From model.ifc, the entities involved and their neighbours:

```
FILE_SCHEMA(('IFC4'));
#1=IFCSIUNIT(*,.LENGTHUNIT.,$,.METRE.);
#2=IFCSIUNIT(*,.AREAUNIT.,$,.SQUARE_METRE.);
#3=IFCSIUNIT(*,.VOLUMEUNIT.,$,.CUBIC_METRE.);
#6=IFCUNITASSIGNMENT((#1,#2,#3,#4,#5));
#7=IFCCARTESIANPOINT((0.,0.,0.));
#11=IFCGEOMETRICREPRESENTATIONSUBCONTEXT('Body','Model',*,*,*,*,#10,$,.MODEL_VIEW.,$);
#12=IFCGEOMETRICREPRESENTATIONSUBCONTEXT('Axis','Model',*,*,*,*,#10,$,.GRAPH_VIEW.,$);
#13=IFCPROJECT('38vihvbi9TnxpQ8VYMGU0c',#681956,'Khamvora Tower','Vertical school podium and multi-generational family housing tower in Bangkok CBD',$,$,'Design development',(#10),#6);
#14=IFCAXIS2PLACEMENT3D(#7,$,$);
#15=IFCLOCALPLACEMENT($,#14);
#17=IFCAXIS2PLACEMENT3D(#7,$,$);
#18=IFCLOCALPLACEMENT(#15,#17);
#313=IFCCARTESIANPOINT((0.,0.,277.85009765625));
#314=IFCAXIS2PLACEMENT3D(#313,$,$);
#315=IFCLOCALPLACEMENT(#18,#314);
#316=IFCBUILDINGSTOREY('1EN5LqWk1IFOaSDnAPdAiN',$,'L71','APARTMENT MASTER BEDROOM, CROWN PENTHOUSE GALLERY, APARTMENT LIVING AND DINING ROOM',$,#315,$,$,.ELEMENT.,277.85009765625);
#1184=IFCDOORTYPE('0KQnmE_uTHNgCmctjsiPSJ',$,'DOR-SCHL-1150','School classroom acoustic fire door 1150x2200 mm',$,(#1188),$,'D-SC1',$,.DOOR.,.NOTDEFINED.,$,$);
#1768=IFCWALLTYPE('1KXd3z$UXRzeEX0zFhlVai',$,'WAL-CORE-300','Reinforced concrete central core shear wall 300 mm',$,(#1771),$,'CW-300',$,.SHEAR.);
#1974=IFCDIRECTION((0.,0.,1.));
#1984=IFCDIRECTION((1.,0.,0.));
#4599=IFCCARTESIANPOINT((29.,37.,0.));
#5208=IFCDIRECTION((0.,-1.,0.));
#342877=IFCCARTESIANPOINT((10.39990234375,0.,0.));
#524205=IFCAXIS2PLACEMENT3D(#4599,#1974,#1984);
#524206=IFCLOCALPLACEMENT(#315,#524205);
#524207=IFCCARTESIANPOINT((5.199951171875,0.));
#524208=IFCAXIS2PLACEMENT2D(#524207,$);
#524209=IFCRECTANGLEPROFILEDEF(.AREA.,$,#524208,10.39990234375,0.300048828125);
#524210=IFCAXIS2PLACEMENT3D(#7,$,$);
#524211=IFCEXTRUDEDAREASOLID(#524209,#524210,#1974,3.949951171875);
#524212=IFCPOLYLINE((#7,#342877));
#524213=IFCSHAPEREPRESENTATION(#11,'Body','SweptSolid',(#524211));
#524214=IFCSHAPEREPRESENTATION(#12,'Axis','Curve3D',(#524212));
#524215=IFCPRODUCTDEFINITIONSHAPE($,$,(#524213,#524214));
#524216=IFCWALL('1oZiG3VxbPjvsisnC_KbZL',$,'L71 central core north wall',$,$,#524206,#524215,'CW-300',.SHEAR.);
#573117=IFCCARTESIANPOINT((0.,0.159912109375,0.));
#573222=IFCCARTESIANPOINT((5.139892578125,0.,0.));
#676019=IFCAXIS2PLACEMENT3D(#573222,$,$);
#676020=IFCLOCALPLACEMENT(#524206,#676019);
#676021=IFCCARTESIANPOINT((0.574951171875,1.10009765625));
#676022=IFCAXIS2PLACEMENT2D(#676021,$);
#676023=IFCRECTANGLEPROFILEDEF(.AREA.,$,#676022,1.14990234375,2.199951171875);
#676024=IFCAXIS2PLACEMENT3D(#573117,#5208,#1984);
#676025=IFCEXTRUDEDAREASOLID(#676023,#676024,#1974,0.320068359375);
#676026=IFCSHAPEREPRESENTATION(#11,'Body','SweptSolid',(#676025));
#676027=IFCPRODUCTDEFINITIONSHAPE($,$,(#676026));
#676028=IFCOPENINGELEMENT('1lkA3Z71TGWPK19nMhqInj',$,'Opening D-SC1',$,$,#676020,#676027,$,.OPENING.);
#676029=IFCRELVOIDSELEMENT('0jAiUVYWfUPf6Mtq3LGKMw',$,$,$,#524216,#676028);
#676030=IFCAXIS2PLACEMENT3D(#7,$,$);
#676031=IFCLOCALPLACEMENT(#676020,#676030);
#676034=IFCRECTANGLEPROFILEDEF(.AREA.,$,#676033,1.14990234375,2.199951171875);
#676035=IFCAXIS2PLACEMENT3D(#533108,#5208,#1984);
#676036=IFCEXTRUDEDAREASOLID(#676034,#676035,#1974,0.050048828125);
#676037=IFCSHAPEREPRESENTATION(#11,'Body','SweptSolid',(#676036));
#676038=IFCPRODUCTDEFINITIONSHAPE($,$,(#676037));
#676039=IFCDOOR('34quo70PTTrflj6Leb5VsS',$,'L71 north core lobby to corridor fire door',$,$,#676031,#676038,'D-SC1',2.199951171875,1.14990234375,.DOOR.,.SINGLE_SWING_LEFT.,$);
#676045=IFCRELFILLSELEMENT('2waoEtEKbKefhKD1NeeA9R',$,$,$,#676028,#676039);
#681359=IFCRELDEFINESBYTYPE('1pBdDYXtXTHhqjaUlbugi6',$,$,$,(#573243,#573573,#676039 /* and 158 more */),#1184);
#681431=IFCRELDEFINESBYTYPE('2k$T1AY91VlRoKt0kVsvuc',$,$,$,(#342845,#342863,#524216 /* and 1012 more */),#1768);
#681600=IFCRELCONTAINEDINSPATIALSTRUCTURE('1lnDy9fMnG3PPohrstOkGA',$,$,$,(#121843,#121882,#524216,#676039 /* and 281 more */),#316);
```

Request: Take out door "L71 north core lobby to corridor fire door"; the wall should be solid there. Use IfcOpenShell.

```python
import ifcopenshell
import ifcopenshell.api.feature
import ifcopenshell.api.root
import ifcopenshell.geom
import ifcopenshell.util.shape

model = ifcopenshell.open("model.ifc")
settings = ifcopenshell.geom.settings()


def volume(element):
    """Net volume in cubic metres, openings subtracted."""
    shape = ifcopenshell.geom.create_shape(settings, element)
    return ifcopenshell.util.shape.get_volume(shape.geometry)


door = model.by_guid("34quo70PTTrflj6Leb5VsS")
opening = door.FillsVoids[0].RelatingOpeningElement
wall = opening.VoidsElements[0].RelatingBuildingElement
before = volume(wall)

ifcopenshell.api.root.remove_product(model, product=door)
ifcopenshell.api.feature.remove_feature(model, feature=opening)

after = volume(wall)

print(f"wall volume {before:.3f} -> {after:.3f} m3")

model.write("model_updated.ifc")
```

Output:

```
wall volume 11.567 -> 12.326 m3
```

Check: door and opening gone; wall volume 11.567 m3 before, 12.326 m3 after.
